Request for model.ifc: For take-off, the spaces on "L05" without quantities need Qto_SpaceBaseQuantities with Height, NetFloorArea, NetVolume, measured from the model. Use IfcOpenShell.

First a look at what the model holds.

```python
import ifcopenshell
import ifcopenshell.util.element
import ifcopenshell.util.unit

model = ifcopenshell.open("model.ifc")
print(model.schema)
for unit_type in ("LENGTHUNIT", "AREAUNIT", "VOLUMEUNIT"):
    print(unit_type, ifcopenshell.util.unit.calculate_unit_scale(model, unit_type))
storey = next(s for s in model.by_type("IfcBuildingStorey") if s.Name == "L05")
spaces = [e for e in ifcopenshell.util.element.get_decomposition(storey) if e.is_a("IfcSpace")]
for e in sorted(spaces, key=lambda e: e.id()):
    print(e.id(), e.is_a(), e.Name, list(ifcopenshell.util.element.get_psets(e, qtos_only=True)), sep=" | ")
```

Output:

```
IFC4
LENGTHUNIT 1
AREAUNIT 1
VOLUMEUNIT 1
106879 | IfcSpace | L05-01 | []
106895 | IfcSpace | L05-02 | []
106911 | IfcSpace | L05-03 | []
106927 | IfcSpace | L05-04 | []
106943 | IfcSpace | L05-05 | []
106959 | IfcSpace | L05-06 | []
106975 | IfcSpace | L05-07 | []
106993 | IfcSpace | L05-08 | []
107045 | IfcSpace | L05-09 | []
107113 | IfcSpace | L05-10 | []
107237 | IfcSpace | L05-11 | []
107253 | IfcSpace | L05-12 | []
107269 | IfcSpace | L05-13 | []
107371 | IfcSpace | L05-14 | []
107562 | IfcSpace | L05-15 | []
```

```python
import ifcopenshell
import ifcopenshell.api.pset
import ifcopenshell.geom
import ifcopenshell.util.element
import ifcopenshell.util.shape
import ifcopenshell.util.unit

model = ifcopenshell.open("model.ifc")
unit_scale = ifcopenshell.util.unit.calculate_unit_scale(model)
area_scale = ifcopenshell.util.unit.calculate_unit_scale(model, "AREAUNIT")
volume_scale = ifcopenshell.util.unit.calculate_unit_scale(model, "VOLUMEUNIT")
settings = ifcopenshell.geom.settings()

storey = next(s for s in model.by_type("IfcBuildingStorey") if s.Name == "L05")
spaces = [e for e in ifcopenshell.util.element.get_decomposition(storey) if e.is_a("IfcSpace")]

for e in sorted(spaces, key=lambda e: e.id()):
    if ifcopenshell.util.element.get_psets(e, qtos_only=True, should_inherit=False):
        continue
    # Geometry comes back in metres, in the element's own axes.
    shape = ifcopenshell.geom.create_shape(settings, e)
    values = {
        "Height": ifcopenshell.util.shape.get_z(shape.geometry) / unit_scale,
        "NetFloorArea": ifcopenshell.util.shape.get_footprint_area(shape.geometry) / area_scale,
        "NetVolume": ifcopenshell.util.shape.get_volume(shape.geometry) / volume_scale,
    }
    qto = ifcopenshell.api.pset.add_qto(model, product=e, name="Qto_SpaceBaseQuantities")
    ifcopenshell.api.pset.edit_qto(model, qto=qto, properties=values)
    print(e.id(), {k: round(v, 3) for k, v in values.items()})

model.write("model_edited.ifc")
```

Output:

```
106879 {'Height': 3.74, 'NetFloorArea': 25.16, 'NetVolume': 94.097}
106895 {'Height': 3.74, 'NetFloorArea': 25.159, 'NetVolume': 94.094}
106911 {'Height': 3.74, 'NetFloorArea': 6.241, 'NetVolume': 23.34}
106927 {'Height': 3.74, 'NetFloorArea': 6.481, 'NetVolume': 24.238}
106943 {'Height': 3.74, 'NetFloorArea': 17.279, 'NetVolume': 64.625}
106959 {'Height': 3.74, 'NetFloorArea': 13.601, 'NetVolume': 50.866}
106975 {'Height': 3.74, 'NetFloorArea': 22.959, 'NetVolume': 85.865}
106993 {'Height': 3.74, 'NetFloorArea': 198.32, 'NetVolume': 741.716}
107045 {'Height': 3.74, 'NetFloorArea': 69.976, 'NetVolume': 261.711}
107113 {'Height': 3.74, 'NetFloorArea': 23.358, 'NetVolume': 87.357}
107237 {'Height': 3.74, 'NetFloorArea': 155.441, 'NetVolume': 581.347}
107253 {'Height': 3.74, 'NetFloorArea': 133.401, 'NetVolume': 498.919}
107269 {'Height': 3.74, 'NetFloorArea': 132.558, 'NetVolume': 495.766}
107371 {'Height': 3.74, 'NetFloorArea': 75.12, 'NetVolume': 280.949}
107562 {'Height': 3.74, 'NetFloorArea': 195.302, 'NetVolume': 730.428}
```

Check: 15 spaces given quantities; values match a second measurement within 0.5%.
